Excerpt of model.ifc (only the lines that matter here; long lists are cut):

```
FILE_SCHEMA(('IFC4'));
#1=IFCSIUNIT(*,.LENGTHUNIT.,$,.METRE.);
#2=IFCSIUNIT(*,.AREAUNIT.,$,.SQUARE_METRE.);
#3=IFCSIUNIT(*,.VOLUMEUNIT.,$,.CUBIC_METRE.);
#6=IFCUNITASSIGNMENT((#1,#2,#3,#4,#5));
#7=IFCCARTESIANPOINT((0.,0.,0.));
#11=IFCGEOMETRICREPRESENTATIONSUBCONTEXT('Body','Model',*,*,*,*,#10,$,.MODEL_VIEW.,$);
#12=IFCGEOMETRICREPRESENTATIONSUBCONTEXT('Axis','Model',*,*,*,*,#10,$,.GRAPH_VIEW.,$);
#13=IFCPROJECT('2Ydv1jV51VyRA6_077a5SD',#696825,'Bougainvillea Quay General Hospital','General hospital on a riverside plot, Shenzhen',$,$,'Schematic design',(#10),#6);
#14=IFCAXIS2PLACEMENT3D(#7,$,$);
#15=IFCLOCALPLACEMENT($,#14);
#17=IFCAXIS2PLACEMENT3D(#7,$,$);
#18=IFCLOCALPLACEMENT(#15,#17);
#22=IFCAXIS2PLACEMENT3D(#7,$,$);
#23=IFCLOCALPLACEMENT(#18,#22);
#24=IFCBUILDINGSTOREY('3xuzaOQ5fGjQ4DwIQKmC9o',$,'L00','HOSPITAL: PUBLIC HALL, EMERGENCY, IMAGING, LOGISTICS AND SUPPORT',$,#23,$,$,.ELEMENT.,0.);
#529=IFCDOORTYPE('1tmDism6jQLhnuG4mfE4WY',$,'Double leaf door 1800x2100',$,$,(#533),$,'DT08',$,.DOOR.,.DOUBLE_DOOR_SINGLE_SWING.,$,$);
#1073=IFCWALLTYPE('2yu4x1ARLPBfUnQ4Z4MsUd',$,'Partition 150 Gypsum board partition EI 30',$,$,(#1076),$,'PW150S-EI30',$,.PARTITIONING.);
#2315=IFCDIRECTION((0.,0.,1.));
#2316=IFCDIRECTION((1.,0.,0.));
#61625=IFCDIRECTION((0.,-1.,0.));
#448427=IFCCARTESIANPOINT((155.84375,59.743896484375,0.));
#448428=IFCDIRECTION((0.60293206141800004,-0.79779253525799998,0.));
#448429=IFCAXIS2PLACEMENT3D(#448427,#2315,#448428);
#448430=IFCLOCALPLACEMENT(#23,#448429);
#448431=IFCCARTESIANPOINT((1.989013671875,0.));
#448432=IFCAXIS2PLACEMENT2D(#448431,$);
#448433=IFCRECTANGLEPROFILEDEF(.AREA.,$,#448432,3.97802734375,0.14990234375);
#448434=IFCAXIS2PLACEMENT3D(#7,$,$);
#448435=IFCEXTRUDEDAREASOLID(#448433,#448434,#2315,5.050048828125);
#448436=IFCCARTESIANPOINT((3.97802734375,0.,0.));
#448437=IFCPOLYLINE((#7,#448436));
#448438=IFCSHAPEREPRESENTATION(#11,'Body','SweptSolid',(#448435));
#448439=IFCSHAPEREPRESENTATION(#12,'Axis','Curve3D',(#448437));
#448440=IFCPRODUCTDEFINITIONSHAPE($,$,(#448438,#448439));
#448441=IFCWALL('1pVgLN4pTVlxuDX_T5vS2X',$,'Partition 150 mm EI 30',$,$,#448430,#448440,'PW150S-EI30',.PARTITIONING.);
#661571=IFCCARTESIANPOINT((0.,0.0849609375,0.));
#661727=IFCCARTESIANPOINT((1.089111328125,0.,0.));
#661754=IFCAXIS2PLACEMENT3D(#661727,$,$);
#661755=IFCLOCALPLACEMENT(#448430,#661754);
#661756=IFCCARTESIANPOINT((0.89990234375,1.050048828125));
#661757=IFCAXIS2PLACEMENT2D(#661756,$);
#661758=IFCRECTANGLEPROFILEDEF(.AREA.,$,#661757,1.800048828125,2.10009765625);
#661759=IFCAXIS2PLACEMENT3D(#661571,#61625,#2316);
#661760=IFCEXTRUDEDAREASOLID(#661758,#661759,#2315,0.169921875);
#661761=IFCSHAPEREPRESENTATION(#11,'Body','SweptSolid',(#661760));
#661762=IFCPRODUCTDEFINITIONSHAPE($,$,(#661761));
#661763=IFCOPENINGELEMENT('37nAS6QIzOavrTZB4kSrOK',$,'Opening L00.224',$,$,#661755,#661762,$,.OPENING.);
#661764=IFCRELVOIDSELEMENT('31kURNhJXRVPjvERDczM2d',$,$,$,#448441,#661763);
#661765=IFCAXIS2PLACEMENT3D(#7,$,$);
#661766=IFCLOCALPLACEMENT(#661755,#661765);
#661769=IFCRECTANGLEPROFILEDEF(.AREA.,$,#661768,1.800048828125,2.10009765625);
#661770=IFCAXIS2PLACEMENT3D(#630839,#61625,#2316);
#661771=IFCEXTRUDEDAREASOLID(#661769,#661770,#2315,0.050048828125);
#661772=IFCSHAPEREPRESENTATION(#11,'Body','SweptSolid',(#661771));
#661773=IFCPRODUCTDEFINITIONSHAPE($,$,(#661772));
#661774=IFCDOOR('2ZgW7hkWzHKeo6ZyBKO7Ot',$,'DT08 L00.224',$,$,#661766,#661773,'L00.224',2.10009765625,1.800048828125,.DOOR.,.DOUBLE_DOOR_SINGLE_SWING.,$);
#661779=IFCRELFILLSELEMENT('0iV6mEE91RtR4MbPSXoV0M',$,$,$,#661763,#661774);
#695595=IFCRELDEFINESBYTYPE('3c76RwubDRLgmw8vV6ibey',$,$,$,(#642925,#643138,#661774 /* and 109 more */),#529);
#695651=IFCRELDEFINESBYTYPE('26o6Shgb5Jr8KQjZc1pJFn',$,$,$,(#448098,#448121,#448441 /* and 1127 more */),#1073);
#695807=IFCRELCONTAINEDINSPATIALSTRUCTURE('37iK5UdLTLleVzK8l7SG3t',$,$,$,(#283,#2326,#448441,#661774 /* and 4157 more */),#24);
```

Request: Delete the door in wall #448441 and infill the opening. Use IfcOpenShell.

```python
import ifcopenshell
import ifcopenshell.api.feature
import ifcopenshell.api.root
import ifcopenshell.geom
import ifcopenshell.util.shape

model = ifcopenshell.open("model.ifc")
settings = ifcopenshell.geom.settings()


def volume(element):
    """Net volume in cubic metres, openings subtracted."""
    shape = ifcopenshell.geom.create_shape(settings, element)
    return ifcopenshell.util.shape.get_volume(shape.geometry)


door = model.by_id(661774)
opening = door.FillsVoids[0].RelatingOpeningElement
wall = opening.VoidsElements[0].RelatingBuildingElement
before = volume(wall)

ifcopenshell.api.root.remove_product(model, product=door)
ifcopenshell.api.feature.remove_feature(model, feature=opening)

after = volume(wall)

print(f"wall volume {before:.3f} -> {after:.3f} m3")

model.write("model_edited.ifc")
```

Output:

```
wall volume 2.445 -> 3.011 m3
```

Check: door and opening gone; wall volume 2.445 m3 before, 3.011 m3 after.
